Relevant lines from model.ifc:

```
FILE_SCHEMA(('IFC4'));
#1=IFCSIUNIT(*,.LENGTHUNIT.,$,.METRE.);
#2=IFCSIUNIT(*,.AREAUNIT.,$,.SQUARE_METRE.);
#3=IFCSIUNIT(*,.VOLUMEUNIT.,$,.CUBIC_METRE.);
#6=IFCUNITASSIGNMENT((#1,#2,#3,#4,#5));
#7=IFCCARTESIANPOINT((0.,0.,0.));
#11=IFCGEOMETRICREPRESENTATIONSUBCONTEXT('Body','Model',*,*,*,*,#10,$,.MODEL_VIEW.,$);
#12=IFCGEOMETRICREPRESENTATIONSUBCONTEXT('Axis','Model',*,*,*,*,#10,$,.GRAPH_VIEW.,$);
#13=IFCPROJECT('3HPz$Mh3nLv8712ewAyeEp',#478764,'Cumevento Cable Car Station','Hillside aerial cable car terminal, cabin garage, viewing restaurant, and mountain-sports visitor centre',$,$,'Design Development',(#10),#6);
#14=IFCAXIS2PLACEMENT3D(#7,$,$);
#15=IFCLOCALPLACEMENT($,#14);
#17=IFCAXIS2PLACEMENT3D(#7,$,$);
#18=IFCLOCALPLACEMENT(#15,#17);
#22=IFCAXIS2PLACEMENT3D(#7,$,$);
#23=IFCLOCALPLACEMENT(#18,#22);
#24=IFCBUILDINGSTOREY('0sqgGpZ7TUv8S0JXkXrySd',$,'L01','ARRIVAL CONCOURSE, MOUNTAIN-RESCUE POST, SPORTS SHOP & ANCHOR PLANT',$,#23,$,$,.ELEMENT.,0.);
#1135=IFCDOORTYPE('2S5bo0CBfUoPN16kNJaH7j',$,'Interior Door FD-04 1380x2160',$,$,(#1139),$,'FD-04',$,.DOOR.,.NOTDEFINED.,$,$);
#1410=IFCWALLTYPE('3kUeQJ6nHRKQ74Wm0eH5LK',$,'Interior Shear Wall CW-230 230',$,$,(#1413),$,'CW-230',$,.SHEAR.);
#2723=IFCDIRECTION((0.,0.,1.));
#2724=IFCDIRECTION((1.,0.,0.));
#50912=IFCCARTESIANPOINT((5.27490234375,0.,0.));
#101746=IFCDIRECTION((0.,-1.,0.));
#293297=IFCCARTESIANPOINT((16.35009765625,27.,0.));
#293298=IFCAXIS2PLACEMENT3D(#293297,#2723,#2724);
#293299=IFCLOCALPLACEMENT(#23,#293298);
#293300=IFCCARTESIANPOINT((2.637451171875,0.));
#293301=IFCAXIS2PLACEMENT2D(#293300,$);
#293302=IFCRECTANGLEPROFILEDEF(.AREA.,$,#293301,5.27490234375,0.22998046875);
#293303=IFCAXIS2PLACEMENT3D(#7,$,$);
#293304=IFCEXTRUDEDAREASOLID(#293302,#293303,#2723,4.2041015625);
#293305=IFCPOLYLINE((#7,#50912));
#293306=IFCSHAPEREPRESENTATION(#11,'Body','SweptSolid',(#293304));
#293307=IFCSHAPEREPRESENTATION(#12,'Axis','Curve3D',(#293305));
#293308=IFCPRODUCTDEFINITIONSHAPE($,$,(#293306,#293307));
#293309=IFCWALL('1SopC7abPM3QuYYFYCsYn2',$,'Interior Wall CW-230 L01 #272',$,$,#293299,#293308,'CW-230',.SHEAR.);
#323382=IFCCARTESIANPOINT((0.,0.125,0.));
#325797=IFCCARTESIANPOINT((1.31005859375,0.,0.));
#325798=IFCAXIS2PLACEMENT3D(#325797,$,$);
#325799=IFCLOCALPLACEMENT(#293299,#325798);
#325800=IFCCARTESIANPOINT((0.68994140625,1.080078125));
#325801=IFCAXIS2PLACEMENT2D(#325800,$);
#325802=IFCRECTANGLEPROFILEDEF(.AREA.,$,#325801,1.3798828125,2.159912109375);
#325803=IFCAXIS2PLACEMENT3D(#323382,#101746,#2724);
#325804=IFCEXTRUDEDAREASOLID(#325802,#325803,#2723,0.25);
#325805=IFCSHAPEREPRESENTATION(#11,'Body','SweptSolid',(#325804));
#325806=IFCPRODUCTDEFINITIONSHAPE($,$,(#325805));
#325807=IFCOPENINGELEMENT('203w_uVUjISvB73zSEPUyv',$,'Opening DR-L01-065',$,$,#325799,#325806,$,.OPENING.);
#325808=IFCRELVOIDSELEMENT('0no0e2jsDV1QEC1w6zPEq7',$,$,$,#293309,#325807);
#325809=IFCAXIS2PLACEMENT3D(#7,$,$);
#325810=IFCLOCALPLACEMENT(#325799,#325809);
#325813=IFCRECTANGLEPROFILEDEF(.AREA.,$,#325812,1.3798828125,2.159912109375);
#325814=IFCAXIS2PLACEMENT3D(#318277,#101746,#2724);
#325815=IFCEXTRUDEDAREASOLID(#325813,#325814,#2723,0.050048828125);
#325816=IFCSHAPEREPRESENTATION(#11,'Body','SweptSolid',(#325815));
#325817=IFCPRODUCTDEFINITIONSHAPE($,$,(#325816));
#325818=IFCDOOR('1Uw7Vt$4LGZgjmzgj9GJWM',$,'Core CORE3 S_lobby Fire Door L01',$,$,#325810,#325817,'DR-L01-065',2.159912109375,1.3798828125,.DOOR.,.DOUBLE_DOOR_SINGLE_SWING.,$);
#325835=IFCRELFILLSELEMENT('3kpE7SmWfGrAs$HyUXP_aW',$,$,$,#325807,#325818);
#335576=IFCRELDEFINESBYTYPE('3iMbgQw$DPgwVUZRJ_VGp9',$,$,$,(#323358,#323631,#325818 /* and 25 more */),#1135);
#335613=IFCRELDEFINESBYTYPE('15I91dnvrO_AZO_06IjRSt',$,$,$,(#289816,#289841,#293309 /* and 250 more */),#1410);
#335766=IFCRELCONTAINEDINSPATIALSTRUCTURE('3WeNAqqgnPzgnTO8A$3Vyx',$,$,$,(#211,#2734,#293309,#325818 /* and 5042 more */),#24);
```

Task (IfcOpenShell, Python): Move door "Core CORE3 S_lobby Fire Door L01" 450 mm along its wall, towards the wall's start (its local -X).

```python
import ifcopenshell
import ifcopenshell.api.geometry
import ifcopenshell.util.placement
import ifcopenshell.util.unit

model = ifcopenshell.open("model.ifc")
unit_scale = ifcopenshell.util.unit.calculate_unit_scale(model)

door = model.by_id(325818)
opening = door.FillsVoids[0].RelatingOpeningElement
wall = opening.VoidsElements[0].RelatingBuildingElement

wall_matrix = ifcopenshell.util.placement.get_local_placement(wall.ObjectPlacement)
shift = wall_matrix[:3, 0] * -0.45 / unit_scale
before = ifcopenshell.util.placement.get_local_placement(door.ObjectPlacement)[:3, 3].copy()

# The door is placed relative to its opening, so it follows when the opening moves.
matrix = ifcopenshell.util.placement.get_local_placement(opening.ObjectPlacement)
matrix[:3, 3] += shift
ifcopenshell.api.geometry.edit_object_placement(
    model, product=opening, matrix=matrix, is_si=False, should_transform_children=True
)

after = ifcopenshell.util.placement.get_local_placement(door.ObjectPlacement)[:3, 3]
print("door moved by", (after - before).round(3) + 0.0)

model.write("model_v2.ifc")
```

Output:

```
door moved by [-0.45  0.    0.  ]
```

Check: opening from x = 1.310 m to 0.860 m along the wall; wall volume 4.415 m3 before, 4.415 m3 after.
